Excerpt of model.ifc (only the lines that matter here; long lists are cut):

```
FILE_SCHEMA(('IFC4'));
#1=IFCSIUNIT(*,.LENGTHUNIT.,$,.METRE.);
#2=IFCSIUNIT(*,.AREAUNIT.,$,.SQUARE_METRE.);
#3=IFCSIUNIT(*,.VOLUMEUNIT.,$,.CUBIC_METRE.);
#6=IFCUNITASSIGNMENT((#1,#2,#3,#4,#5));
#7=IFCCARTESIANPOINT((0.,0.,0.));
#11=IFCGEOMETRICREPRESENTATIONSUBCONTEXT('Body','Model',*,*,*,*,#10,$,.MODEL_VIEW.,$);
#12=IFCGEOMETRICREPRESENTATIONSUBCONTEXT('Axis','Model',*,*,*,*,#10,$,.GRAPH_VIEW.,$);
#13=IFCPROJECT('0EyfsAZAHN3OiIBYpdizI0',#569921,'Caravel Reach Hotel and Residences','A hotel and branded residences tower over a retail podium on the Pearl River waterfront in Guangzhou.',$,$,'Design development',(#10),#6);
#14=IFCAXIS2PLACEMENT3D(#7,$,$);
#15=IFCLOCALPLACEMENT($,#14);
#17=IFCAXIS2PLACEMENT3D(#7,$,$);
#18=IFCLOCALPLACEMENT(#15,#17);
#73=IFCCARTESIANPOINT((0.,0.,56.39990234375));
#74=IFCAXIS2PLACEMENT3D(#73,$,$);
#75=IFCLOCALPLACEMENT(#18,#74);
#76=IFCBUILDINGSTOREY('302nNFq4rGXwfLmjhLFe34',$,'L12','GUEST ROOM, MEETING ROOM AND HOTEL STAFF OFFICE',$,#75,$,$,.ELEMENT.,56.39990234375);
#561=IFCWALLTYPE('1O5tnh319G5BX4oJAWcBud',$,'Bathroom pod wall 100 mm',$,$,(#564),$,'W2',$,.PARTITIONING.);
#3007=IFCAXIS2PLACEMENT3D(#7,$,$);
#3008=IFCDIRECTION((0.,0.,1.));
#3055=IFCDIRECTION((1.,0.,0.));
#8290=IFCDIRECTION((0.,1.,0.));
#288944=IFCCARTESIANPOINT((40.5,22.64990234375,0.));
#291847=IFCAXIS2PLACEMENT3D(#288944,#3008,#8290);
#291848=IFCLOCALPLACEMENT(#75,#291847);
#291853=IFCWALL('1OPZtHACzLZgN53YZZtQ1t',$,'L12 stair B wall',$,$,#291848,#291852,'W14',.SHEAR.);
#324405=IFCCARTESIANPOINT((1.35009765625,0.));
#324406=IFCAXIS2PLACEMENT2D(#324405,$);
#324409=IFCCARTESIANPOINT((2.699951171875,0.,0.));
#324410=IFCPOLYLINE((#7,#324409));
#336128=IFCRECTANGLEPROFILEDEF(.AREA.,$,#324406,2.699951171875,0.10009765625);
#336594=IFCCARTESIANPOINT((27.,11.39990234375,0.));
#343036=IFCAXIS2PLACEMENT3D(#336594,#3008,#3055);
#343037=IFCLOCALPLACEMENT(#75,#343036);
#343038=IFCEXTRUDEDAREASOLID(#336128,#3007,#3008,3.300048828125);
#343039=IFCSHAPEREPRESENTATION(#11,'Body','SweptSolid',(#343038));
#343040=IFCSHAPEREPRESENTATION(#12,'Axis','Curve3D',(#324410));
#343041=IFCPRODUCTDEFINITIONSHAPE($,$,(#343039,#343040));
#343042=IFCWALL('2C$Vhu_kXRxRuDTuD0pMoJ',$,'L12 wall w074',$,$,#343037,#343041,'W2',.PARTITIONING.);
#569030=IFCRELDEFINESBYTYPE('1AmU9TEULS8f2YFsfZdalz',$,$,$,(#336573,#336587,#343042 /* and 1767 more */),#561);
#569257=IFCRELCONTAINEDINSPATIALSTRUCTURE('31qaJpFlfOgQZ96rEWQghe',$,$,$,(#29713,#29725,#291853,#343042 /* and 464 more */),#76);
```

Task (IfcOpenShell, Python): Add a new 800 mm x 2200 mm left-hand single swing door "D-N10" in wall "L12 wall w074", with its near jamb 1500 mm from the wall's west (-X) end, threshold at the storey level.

```python
import numpy as np
import ifcopenshell
import ifcopenshell.api.feature
import ifcopenshell.api.geometry
import ifcopenshell.api.root
import ifcopenshell.api.spatial
import ifcopenshell.geom
import ifcopenshell.util.element
import ifcopenshell.util.placement
import ifcopenshell.util.representation
import ifcopenshell.util.shape
import ifcopenshell.util.unit

model = ifcopenshell.open("model.ifc")
unit_scale = ifcopenshell.util.unit.calculate_unit_scale(model)
settings = ifcopenshell.geom.settings()


def volume(element):
    """Net volume in cubic metres, openings subtracted."""
    shape = ifcopenshell.geom.create_shape(settings, element)
    return ifcopenshell.util.shape.get_volume(shape.geometry)


wall = model.by_guid("2C$Vhu_kXRxRuDTuD0pMoJ")
storey = ifcopenshell.util.element.get_container(wall, ifc_class="IfcBuildingStorey")
context = ifcopenshell.util.representation.get_context(model, "Model", "Body", "MODEL_VIEW")
before = volume(wall)

width, height, from_end, sill = 0.8, 2.2, 1.5, 0.0  # metres

# The wall runs along its own X axis, and the end named is its -X end.
wall_shape = ifcopenshell.geom.create_shape(settings, wall)
x, y, z = ifcopenshell.util.shape.get_vertices(wall_shape.geometry).T
start = x.min() + from_end
face, thickness = float(y.min()), float(y.max() - y.min())
wall_matrix = ifcopenshell.util.placement.get_local_placement(wall.ObjectPlacement)
level = ifcopenshell.util.placement.get_local_placement(storey.ObjectPlacement)[2, 3]


def in_wall(x, y):
    """Placement at x, y metres in the wall's axes, at sill height."""
    matrix = wall_matrix.copy()
    matrix[:, 3] = wall_matrix @ np.array([x / unit_scale, y / unit_scale, 0.0, 1.0])
    matrix[2, 3] = level + sill / unit_scale
    return matrix


# Opening: a box that overshoots both wall faces by 50 mm.
opening = ifcopenshell.api.root.create_entity(model, ifc_class="IfcOpeningElement", predefined_type="OPENING")
box = ifcopenshell.api.geometry.add_wall_representation(
    model, context=context, length=width, height=height, thickness=thickness + 0.1
)
ifcopenshell.api.geometry.assign_representation(model, product=opening, representation=box)
ifcopenshell.api.geometry.edit_object_placement(model, product=opening, matrix=in_wall(start, face - 0.05), is_si=False)
ifcopenshell.api.feature.add_feature(model, feature=opening, element=wall)

door = ifcopenshell.api.root.create_entity(model, ifc_class="IfcDoor", name="D-N10", predefined_type="DOOR")
door.OverallWidth, door.OverallHeight = width / unit_scale, height / unit_scale
door.OperationType = "SINGLE_SWING_LEFT"
body = ifcopenshell.api.geometry.add_door_representation(
    model,
    context=context,
    overall_width=door.OverallWidth,
    overall_height=door.OverallHeight,
    operation_type="SINGLE_SWING_LEFT",
    lining_properties={"LiningDepth": thickness / unit_scale, "ThresholdDepth": thickness / unit_scale},
)
ifcopenshell.api.geometry.assign_representation(model, product=door, representation=body)
ifcopenshell.api.spatial.assign_container(model, products=[door], relating_structure=storey)
ifcopenshell.api.feature.add_filling(model, opening=opening, element=door)

# The lining spans the wall, so the door starts at the wall face.
ifcopenshell.api.geometry.edit_object_placement(model, product=door, matrix=in_wall(start, face), is_si=False)

after = volume(wall)

print(f"wall volume {before:.3f} -> {after:.3f} m3")

model.write("model_updated.ifc")
```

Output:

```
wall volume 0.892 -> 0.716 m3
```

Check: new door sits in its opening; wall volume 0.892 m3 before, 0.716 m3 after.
